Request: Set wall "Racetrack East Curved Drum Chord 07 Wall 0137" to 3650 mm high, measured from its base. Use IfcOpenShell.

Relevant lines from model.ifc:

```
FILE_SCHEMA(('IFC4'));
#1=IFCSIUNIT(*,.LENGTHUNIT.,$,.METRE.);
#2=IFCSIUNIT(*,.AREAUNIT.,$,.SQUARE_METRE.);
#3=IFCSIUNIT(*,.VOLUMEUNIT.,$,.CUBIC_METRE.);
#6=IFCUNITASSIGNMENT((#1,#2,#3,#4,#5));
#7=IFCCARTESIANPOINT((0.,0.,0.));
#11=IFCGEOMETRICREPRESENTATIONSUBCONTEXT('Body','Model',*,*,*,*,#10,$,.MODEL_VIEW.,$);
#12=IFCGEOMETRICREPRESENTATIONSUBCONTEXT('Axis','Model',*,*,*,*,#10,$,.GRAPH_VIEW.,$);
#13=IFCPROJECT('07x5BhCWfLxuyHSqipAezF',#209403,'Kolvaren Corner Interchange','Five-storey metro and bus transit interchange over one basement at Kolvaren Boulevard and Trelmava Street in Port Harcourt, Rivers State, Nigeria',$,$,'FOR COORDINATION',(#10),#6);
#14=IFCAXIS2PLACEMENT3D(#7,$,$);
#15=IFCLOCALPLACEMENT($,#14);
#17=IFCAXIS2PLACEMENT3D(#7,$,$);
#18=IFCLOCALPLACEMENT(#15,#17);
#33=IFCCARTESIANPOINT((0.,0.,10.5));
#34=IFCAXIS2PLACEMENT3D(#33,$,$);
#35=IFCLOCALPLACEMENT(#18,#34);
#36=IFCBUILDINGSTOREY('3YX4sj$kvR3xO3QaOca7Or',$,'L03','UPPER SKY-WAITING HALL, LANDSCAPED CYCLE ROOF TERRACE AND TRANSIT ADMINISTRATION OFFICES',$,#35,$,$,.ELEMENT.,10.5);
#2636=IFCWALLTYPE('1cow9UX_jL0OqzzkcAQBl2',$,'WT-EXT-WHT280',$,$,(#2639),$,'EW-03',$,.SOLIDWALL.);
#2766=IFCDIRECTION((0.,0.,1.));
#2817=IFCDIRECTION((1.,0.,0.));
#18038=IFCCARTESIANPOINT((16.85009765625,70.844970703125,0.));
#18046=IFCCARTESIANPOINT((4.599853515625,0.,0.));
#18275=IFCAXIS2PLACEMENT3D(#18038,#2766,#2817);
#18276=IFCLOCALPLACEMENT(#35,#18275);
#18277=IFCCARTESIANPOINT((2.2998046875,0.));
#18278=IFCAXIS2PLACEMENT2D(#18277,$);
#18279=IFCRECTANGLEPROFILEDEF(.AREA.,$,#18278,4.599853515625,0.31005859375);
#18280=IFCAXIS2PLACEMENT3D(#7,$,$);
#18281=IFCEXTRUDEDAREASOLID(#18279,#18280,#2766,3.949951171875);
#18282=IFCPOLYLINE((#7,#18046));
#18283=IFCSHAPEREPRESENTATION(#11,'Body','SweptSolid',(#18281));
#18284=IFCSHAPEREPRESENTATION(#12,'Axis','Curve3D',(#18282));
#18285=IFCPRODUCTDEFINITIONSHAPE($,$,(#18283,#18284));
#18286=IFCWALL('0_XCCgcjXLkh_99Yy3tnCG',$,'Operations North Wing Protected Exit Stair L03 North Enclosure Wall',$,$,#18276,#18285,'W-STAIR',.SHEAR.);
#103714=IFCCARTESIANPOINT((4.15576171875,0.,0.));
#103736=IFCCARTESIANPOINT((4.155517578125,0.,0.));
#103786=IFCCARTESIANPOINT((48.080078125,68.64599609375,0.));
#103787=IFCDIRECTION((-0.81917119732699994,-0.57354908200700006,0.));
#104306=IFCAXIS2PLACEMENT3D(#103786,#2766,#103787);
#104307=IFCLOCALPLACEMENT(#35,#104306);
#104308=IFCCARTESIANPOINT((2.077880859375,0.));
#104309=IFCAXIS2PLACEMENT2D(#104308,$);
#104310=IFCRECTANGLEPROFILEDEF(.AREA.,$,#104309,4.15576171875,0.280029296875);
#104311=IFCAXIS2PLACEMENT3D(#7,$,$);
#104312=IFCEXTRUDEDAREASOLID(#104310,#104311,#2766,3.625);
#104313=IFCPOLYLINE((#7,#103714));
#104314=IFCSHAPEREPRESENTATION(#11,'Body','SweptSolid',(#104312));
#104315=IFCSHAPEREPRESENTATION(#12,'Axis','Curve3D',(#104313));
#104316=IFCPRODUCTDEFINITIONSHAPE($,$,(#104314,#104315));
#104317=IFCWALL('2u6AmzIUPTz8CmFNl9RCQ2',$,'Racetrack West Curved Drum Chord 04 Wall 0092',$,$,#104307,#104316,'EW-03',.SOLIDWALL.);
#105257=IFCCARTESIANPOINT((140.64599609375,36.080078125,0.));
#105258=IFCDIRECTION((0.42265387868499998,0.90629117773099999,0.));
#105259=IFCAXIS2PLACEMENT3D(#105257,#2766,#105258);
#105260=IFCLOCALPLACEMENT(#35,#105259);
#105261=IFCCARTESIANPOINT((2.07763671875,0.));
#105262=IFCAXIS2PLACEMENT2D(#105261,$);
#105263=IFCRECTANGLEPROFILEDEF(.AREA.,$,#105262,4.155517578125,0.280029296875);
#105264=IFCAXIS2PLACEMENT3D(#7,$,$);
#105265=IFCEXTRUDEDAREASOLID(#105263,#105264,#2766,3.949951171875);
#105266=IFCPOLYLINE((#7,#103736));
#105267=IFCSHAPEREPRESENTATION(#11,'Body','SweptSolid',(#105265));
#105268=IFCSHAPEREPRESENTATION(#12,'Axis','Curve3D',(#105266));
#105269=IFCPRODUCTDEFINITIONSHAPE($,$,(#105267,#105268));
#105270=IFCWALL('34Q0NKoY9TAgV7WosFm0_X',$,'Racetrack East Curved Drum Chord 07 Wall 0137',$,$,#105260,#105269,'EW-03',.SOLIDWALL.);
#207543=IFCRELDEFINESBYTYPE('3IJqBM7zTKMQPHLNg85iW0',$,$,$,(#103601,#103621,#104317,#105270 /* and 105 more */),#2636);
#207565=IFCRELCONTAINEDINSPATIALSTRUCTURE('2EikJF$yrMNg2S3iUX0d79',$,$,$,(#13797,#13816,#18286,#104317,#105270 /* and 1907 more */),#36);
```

```python
import ifcopenshell
import ifcopenshell.geom
import ifcopenshell.util.representation
import ifcopenshell.util.shape
import ifcopenshell.util.unit

model = ifcopenshell.open("model.ifc")
unit_scale = ifcopenshell.util.unit.calculate_unit_scale(model)
settings = ifcopenshell.geom.settings()


def volume(element):
    """Net volume in cubic metres, openings subtracted."""
    shape = ifcopenshell.geom.create_shape(settings, element)
    return ifcopenshell.util.shape.get_volume(shape.geometry)


wall = model.by_guid("34Q0NKoY9TAgV7WosFm0_X")
before = volume(wall)

body = ifcopenshell.util.representation.get_representation(wall, "Model", "Body")
solid = body.Items[0]
old_height = solid.Depth
solid.Depth = 3.65 / unit_scale
after = volume(wall)

print(f"height {old_height:g} -> {solid.Depth:g}, volume {before:.3f} -> {after:.3f} m3")

model.write("model_v2.ifc")
```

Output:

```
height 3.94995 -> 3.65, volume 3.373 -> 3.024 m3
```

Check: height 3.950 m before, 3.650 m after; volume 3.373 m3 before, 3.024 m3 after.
